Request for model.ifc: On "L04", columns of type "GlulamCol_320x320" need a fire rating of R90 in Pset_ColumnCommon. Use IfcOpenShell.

First a look at what the model holds.

```python
import ifcopenshell
import ifcopenshell.util.element

model = ifcopenshell.open("model.ifc")
print(model.schema)
storey = next(s for s in model.by_type("IfcBuildingStorey") if s.Name == "L04")
columns = [e for e in ifcopenshell.util.element.get_decomposition(storey) if e.is_a("IfcColumn")]
seen = {}
for e in columns:
    element_type = ifcopenshell.util.element.get_type(e)
    key = (element_type.Name if element_type != e and element_type else None, ifcopenshell.util.element.get_pset(e, "Pset_ColumnCommon", "FireRating"))
    seen[key] = seen.get(key, 0) + 1
for (name, value), count in sorted(seen.items(), key=str):
    print(count, "x", name, "|", value)
```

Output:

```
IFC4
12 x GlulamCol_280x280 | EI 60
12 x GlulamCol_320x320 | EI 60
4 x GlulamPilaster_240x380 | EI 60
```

```python
import ifcopenshell
import ifcopenshell.api.pset
import ifcopenshell.util.element

model = ifcopenshell.open("model.ifc")

storey = next(s for s in model.by_type("IfcBuildingStorey") if s.Name == "L04")
columns = [e for e in ifcopenshell.util.element.get_decomposition(storey) if e.is_a("IfcColumn")]

count = 0
for e in columns:
    element_type = ifcopenshell.util.element.get_type(e)
    if element_type in (None, e) or element_type.Name != "GlulamCol_320x320":
        continue
    # add_pset returns the element's existing set when there is one.
    pset = ifcopenshell.api.pset.add_pset(model, product=e, name="Pset_ColumnCommon")
    ifcopenshell.api.pset.edit_pset(model, pset=pset, properties={"FireRating": "R90"})
    count += 1

print(count, "columns updated")

model.write("model_updated.ifc")
```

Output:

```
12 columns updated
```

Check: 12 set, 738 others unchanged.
